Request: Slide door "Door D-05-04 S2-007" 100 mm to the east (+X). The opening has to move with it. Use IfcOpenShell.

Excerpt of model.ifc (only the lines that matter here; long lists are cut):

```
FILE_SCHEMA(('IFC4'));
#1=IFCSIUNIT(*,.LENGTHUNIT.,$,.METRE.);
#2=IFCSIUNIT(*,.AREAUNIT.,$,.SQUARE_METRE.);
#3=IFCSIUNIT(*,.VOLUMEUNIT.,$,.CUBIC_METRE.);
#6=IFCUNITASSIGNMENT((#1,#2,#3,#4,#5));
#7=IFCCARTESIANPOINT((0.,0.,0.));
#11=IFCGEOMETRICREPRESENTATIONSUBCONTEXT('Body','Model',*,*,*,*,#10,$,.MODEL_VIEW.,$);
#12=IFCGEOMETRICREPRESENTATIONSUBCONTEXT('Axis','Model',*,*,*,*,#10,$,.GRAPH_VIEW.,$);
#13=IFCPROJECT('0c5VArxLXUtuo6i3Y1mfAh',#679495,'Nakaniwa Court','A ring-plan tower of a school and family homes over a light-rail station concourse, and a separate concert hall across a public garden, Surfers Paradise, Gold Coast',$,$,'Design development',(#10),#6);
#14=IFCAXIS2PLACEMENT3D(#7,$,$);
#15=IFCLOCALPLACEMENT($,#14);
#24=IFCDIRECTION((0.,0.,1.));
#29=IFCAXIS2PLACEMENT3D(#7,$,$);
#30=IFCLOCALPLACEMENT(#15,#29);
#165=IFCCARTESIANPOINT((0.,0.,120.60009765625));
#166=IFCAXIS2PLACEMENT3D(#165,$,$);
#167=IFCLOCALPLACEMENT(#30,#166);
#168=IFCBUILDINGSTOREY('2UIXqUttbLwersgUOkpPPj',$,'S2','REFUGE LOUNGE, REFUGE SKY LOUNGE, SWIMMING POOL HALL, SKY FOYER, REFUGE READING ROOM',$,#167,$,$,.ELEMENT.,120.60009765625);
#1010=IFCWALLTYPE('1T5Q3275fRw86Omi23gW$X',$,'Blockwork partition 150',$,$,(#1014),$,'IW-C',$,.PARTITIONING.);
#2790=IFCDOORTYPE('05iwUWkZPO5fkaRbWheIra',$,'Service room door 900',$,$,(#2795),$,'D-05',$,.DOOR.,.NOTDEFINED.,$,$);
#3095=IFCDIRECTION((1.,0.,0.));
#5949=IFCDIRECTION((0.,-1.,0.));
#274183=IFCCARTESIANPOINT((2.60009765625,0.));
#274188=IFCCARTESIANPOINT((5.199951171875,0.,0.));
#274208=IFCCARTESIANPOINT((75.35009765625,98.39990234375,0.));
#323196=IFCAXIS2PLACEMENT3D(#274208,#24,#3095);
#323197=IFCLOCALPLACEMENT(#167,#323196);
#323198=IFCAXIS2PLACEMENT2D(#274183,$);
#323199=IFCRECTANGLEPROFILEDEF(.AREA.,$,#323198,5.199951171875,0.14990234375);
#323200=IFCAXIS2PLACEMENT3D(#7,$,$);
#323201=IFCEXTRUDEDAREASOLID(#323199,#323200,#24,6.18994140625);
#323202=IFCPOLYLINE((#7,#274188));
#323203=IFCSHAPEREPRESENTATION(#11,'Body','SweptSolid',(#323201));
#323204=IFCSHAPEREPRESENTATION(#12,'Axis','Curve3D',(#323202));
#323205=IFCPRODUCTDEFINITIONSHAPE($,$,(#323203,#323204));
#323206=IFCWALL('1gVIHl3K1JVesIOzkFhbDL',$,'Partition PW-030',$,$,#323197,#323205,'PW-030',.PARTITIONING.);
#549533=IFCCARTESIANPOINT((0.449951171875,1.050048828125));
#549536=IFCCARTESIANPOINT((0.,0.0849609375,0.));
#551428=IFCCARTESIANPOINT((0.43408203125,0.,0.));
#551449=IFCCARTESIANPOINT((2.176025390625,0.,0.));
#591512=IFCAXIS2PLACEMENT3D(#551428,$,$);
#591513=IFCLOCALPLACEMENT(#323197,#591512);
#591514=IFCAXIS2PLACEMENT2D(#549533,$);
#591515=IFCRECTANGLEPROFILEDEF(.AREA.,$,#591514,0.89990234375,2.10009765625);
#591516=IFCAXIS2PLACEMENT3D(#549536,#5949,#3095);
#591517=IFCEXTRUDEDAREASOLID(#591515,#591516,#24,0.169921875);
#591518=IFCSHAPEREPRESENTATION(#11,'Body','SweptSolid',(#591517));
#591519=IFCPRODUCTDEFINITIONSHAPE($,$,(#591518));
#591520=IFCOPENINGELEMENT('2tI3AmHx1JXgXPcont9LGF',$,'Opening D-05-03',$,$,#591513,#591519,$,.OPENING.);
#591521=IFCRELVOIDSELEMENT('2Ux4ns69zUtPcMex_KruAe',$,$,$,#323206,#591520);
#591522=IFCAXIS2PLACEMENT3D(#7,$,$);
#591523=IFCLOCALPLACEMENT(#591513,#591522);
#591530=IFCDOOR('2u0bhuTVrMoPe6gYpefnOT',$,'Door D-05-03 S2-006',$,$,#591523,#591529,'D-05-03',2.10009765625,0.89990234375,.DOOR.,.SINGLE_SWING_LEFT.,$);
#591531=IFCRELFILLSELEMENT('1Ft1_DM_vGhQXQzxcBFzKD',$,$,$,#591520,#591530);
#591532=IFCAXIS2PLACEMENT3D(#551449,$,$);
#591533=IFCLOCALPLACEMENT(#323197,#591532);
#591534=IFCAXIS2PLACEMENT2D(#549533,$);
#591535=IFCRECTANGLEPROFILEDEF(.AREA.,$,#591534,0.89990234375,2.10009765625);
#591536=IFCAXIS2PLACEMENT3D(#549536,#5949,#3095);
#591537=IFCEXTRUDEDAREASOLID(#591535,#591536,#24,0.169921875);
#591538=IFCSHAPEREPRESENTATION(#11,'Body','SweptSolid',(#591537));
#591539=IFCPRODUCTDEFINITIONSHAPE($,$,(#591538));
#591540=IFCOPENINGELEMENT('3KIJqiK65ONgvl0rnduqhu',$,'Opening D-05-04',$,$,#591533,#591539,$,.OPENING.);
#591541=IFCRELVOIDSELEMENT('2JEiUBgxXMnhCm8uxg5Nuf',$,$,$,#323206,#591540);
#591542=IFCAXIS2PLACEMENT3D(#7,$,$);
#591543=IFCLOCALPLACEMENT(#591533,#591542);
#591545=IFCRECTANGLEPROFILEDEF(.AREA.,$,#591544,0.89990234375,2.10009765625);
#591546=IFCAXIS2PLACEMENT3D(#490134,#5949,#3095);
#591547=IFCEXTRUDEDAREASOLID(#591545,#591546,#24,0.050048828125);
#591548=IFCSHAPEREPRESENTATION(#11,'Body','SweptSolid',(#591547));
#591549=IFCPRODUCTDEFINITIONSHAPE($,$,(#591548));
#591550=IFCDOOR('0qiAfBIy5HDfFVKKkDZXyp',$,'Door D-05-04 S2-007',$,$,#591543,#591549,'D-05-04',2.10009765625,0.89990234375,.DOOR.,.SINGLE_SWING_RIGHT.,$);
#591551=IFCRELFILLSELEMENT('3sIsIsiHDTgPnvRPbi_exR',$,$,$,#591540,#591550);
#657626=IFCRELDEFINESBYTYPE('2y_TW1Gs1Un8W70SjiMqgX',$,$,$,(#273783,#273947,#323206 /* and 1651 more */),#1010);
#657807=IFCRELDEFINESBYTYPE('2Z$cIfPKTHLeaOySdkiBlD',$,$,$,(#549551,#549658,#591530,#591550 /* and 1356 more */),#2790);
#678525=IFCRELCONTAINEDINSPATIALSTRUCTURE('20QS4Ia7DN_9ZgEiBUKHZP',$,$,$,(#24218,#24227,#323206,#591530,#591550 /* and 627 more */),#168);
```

```python
import ifcopenshell
import ifcopenshell.api.geometry
import ifcopenshell.util.placement
import ifcopenshell.util.unit

model = ifcopenshell.open("model.ifc")
unit_scale = ifcopenshell.util.unit.calculate_unit_scale(model)

door = model.by_guid("0qiAfBIy5HDfFVKKkDZXyp")
opening = door.FillsVoids[0].RelatingOpeningElement
wall = opening.VoidsElements[0].RelatingBuildingElement

wall_matrix = ifcopenshell.util.placement.get_local_placement(wall.ObjectPlacement)
shift = wall_matrix[:3, 0] * 0.1 / unit_scale
before = ifcopenshell.util.placement.get_local_placement(door.ObjectPlacement)[:3, 3].copy()

# The door is placed relative to its opening, so it follows when the opening moves.
matrix = ifcopenshell.util.placement.get_local_placement(opening.ObjectPlacement)
matrix[:3, 3] += shift
ifcopenshell.api.geometry.edit_object_placement(
    model, product=opening, matrix=matrix, is_si=False, should_transform_children=True
)

after = ifcopenshell.util.placement.get_local_placement(door.ObjectPlacement)[:3, 3]
print("door moved by", (after - before).round(3) + 0.0)

model.write("model_updated.ifc")
```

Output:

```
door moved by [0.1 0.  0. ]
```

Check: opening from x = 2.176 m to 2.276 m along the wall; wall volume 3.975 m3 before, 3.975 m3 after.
